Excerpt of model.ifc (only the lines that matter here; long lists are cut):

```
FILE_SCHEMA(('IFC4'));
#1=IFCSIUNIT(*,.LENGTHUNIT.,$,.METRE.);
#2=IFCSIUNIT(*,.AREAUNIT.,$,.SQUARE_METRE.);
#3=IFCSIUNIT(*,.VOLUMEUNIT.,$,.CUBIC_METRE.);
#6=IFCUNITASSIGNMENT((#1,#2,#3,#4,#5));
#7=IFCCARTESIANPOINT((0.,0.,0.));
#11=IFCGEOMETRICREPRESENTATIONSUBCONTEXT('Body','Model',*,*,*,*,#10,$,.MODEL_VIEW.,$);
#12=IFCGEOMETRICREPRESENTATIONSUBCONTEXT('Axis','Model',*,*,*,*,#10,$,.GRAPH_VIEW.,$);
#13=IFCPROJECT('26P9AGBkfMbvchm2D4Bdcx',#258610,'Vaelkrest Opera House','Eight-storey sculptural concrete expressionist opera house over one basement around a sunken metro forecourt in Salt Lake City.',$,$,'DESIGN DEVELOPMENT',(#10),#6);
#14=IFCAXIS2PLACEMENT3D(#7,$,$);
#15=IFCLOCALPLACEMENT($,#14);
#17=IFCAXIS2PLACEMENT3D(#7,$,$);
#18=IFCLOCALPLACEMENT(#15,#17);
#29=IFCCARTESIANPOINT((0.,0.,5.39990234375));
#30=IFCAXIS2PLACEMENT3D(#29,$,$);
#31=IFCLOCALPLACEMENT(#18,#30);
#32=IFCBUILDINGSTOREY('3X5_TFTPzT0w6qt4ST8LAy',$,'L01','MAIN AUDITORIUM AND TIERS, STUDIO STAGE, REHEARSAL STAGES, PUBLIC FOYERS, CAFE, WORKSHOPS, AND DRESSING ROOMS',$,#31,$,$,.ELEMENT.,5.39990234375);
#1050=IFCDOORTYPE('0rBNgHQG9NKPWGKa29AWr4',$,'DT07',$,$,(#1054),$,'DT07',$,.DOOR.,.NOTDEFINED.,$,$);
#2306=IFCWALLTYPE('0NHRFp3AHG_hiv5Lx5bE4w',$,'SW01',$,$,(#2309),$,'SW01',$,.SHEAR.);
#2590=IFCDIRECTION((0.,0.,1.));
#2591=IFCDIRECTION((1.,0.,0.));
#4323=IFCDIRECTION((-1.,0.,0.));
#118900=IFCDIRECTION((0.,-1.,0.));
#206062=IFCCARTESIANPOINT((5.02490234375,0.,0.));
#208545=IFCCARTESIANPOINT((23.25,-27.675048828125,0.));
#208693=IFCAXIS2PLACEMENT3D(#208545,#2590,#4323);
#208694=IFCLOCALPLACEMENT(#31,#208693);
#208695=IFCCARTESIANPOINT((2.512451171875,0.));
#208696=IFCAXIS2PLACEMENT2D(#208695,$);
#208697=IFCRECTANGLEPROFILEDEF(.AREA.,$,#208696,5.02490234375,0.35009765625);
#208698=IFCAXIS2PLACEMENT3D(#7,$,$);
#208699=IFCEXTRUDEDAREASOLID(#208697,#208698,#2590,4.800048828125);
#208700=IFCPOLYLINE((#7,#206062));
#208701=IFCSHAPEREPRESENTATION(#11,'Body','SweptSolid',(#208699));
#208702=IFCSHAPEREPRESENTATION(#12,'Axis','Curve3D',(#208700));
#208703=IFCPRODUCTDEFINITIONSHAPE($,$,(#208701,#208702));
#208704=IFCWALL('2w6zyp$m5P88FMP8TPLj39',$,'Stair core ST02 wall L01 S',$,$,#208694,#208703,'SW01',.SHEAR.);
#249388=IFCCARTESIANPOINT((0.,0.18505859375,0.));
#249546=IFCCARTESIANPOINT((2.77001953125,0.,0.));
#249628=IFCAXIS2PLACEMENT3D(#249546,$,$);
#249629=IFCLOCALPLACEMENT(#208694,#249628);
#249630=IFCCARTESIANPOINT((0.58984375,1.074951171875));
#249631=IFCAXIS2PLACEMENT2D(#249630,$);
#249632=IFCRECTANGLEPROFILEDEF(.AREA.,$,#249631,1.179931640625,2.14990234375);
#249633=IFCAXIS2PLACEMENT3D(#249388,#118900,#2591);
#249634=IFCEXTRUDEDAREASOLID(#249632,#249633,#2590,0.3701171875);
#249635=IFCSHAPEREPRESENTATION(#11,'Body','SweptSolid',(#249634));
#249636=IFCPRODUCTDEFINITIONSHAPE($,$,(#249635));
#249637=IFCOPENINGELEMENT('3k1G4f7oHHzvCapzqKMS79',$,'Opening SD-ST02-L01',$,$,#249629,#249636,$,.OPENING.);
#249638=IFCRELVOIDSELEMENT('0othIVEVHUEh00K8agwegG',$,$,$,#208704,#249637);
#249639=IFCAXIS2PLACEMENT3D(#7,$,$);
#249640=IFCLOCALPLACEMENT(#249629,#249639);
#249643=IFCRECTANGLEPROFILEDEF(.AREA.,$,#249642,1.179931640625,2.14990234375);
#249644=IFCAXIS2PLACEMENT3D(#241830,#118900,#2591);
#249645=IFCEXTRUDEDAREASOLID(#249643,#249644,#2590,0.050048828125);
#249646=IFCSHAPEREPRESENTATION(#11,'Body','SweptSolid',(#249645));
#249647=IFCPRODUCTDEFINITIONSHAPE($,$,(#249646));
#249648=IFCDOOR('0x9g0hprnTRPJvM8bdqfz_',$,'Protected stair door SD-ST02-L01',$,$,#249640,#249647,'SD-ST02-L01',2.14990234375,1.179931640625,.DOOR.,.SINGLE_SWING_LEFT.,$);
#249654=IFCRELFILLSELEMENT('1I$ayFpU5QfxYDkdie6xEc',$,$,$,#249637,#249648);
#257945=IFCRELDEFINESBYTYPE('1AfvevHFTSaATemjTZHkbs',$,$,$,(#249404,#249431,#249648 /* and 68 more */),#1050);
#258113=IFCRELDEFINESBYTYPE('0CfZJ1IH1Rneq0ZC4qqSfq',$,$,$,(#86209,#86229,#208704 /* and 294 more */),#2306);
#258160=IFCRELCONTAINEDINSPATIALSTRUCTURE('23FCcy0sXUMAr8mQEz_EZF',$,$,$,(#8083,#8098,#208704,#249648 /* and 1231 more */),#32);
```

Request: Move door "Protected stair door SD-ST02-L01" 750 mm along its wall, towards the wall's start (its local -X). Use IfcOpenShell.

```python
import ifcopenshell
import ifcopenshell.api.geometry
import ifcopenshell.util.placement

model = ifcopenshell.open("model.ifc")

door = model.by_id(249648)
opening = door.FillsVoids[0].RelatingOpeningElement
wall = opening.VoidsElements[0].RelatingBuildingElement

wall_matrix = ifcopenshell.util.placement.get_local_placement(wall.ObjectPlacement)
shift = wall_matrix[:3, 0] * -0.75
before = ifcopenshell.util.placement.get_local_placement(door.ObjectPlacement)[:3, 3].copy()

# The door is placed relative to its opening, so it follows when the opening moves.
matrix = ifcopenshell.util.placement.get_local_placement(opening.ObjectPlacement)
matrix[:3, 3] += shift
ifcopenshell.api.geometry.edit_object_placement(
    model, product=opening, matrix=matrix, is_si=False, should_transform_children=True
)

after = ifcopenshell.util.placement.get_local_placement(door.ObjectPlacement)[:3, 3]
print("door moved by", (after - before).round(3) + 0.0)

model.write("model_updated.ifc")
```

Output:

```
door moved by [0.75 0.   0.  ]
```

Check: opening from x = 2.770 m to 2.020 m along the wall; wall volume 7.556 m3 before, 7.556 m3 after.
